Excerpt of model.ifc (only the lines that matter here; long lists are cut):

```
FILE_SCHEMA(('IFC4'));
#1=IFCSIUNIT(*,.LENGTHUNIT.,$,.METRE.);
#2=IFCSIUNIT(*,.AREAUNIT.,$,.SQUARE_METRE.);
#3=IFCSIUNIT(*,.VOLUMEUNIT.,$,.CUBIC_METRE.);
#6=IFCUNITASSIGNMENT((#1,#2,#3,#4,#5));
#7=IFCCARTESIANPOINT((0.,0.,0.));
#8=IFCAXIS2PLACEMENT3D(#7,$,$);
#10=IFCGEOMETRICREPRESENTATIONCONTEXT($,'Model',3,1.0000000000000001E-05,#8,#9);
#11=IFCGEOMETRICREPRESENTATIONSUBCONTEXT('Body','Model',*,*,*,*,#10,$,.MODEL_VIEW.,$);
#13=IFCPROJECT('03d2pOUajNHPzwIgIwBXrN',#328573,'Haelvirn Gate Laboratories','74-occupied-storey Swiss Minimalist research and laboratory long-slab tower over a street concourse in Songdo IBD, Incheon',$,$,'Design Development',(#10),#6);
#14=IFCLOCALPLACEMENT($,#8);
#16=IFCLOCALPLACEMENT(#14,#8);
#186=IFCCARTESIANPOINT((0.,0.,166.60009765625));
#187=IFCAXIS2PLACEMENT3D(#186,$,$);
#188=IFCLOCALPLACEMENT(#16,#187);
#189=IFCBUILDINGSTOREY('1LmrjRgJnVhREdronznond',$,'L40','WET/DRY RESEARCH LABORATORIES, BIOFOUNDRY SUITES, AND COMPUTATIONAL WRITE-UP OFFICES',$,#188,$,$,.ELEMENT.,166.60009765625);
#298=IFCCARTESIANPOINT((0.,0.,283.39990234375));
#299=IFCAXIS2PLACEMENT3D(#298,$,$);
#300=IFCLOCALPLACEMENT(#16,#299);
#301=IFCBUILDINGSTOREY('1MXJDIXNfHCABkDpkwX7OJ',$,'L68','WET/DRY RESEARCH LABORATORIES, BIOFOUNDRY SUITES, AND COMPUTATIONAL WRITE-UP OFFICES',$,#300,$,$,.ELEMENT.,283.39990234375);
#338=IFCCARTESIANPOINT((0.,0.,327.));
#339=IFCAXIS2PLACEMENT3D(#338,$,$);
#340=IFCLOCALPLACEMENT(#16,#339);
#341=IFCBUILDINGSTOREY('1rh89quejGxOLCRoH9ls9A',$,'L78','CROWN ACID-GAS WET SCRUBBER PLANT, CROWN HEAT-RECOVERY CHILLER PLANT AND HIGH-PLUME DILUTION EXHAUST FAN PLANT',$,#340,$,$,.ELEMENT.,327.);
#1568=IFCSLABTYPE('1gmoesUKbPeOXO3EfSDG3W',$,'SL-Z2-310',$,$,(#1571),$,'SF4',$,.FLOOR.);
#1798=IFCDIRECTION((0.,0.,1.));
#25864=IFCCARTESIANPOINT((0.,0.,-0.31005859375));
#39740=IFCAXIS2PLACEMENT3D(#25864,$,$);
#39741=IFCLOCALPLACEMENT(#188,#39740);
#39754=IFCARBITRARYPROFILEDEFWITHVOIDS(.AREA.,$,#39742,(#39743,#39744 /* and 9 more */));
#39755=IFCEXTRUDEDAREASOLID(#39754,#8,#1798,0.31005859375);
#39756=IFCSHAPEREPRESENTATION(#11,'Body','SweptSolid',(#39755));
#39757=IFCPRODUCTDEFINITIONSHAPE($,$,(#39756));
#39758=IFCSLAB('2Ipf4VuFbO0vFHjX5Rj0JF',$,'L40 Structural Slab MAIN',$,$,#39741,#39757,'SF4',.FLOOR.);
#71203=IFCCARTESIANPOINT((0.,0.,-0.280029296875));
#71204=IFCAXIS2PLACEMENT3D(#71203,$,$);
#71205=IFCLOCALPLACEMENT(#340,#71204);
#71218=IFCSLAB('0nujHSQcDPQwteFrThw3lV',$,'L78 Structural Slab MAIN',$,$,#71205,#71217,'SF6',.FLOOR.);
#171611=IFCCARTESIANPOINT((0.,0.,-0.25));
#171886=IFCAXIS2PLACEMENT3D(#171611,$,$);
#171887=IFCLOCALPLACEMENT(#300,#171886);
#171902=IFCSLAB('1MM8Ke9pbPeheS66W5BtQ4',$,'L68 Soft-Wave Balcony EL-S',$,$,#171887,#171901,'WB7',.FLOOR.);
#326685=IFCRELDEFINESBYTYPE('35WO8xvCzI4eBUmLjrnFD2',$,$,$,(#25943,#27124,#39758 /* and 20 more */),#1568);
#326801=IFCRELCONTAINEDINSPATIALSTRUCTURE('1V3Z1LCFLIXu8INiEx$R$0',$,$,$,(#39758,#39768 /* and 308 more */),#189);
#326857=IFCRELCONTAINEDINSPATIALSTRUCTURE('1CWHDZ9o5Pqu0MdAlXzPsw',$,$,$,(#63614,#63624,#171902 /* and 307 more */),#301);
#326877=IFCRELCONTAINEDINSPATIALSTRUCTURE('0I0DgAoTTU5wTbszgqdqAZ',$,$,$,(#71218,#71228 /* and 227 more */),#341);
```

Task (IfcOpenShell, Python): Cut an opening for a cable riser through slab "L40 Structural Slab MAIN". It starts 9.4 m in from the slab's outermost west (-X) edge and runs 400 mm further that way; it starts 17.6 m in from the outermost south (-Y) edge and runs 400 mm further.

```python
import numpy as np
import ifcopenshell
import ifcopenshell.api.feature
import ifcopenshell.api.geometry
import ifcopenshell.api.root
import ifcopenshell.geom
import ifcopenshell.util.placement
import ifcopenshell.util.representation
import ifcopenshell.util.shape
import ifcopenshell.util.unit

model = ifcopenshell.open("model.ifc")
unit_scale = ifcopenshell.util.unit.calculate_unit_scale(model)
settings = ifcopenshell.geom.settings()


def volume(element):
    """Net volume in cubic metres, openings subtracted."""
    shape = ifcopenshell.geom.create_shape(settings, element)
    return ifcopenshell.util.shape.get_volume(shape.geometry)


slab = model.by_guid("2Ipf4VuFbO0vFHjX5Rj0JF")
before = volume(slab)

# Extent in the slab's own axes, in metres. The edges named are its -X and -Y sides.
slab_shape = ifcopenshell.geom.create_shape(settings, slab)
vertices = ifcopenshell.util.shape.get_vertices(slab_shape.geometry)
x_min, y_min, bottom = vertices.min(axis=0)
top = vertices[:, 2].max()

opening = ifcopenshell.api.root.create_entity(model, ifc_class="IfcOpeningElement", name="Cable riser opening", predefined_type="OPENING")
context = ifcopenshell.util.representation.get_context(model, "Model", "Body", "MODEL_VIEW")
width, depth = 0.4, 0.4
outline = [(0.0, 0.0), (width, 0.0), (width, depth), (0.0, depth), (0.0, 0.0)]
# Overshoot both faces by 50 mm so the cut is clean.
shape = ifcopenshell.api.geometry.add_slab_representation(
    model, context=context, depth=top - bottom + 0.1, polyline=outline
)
ifcopenshell.api.geometry.assign_representation(model, product=opening, representation=shape)

matrix = ifcopenshell.util.placement.get_local_placement(slab.ObjectPlacement)
matrix[:, 3] = matrix @ np.append(np.array([x_min + 9.4, y_min + 17.6, bottom - 0.05]) / unit_scale, 1.0)
ifcopenshell.api.geometry.edit_object_placement(model, product=opening, matrix=matrix, is_si=False)
ifcopenshell.api.feature.add_feature(model, feature=opening, element=slab)

after = volume(slab)

print(f"slab volume {before:.3f} -> {after:.3f} m3")

model.write("model_rev.ifc")
```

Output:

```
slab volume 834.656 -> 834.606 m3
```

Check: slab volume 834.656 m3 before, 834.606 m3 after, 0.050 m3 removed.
